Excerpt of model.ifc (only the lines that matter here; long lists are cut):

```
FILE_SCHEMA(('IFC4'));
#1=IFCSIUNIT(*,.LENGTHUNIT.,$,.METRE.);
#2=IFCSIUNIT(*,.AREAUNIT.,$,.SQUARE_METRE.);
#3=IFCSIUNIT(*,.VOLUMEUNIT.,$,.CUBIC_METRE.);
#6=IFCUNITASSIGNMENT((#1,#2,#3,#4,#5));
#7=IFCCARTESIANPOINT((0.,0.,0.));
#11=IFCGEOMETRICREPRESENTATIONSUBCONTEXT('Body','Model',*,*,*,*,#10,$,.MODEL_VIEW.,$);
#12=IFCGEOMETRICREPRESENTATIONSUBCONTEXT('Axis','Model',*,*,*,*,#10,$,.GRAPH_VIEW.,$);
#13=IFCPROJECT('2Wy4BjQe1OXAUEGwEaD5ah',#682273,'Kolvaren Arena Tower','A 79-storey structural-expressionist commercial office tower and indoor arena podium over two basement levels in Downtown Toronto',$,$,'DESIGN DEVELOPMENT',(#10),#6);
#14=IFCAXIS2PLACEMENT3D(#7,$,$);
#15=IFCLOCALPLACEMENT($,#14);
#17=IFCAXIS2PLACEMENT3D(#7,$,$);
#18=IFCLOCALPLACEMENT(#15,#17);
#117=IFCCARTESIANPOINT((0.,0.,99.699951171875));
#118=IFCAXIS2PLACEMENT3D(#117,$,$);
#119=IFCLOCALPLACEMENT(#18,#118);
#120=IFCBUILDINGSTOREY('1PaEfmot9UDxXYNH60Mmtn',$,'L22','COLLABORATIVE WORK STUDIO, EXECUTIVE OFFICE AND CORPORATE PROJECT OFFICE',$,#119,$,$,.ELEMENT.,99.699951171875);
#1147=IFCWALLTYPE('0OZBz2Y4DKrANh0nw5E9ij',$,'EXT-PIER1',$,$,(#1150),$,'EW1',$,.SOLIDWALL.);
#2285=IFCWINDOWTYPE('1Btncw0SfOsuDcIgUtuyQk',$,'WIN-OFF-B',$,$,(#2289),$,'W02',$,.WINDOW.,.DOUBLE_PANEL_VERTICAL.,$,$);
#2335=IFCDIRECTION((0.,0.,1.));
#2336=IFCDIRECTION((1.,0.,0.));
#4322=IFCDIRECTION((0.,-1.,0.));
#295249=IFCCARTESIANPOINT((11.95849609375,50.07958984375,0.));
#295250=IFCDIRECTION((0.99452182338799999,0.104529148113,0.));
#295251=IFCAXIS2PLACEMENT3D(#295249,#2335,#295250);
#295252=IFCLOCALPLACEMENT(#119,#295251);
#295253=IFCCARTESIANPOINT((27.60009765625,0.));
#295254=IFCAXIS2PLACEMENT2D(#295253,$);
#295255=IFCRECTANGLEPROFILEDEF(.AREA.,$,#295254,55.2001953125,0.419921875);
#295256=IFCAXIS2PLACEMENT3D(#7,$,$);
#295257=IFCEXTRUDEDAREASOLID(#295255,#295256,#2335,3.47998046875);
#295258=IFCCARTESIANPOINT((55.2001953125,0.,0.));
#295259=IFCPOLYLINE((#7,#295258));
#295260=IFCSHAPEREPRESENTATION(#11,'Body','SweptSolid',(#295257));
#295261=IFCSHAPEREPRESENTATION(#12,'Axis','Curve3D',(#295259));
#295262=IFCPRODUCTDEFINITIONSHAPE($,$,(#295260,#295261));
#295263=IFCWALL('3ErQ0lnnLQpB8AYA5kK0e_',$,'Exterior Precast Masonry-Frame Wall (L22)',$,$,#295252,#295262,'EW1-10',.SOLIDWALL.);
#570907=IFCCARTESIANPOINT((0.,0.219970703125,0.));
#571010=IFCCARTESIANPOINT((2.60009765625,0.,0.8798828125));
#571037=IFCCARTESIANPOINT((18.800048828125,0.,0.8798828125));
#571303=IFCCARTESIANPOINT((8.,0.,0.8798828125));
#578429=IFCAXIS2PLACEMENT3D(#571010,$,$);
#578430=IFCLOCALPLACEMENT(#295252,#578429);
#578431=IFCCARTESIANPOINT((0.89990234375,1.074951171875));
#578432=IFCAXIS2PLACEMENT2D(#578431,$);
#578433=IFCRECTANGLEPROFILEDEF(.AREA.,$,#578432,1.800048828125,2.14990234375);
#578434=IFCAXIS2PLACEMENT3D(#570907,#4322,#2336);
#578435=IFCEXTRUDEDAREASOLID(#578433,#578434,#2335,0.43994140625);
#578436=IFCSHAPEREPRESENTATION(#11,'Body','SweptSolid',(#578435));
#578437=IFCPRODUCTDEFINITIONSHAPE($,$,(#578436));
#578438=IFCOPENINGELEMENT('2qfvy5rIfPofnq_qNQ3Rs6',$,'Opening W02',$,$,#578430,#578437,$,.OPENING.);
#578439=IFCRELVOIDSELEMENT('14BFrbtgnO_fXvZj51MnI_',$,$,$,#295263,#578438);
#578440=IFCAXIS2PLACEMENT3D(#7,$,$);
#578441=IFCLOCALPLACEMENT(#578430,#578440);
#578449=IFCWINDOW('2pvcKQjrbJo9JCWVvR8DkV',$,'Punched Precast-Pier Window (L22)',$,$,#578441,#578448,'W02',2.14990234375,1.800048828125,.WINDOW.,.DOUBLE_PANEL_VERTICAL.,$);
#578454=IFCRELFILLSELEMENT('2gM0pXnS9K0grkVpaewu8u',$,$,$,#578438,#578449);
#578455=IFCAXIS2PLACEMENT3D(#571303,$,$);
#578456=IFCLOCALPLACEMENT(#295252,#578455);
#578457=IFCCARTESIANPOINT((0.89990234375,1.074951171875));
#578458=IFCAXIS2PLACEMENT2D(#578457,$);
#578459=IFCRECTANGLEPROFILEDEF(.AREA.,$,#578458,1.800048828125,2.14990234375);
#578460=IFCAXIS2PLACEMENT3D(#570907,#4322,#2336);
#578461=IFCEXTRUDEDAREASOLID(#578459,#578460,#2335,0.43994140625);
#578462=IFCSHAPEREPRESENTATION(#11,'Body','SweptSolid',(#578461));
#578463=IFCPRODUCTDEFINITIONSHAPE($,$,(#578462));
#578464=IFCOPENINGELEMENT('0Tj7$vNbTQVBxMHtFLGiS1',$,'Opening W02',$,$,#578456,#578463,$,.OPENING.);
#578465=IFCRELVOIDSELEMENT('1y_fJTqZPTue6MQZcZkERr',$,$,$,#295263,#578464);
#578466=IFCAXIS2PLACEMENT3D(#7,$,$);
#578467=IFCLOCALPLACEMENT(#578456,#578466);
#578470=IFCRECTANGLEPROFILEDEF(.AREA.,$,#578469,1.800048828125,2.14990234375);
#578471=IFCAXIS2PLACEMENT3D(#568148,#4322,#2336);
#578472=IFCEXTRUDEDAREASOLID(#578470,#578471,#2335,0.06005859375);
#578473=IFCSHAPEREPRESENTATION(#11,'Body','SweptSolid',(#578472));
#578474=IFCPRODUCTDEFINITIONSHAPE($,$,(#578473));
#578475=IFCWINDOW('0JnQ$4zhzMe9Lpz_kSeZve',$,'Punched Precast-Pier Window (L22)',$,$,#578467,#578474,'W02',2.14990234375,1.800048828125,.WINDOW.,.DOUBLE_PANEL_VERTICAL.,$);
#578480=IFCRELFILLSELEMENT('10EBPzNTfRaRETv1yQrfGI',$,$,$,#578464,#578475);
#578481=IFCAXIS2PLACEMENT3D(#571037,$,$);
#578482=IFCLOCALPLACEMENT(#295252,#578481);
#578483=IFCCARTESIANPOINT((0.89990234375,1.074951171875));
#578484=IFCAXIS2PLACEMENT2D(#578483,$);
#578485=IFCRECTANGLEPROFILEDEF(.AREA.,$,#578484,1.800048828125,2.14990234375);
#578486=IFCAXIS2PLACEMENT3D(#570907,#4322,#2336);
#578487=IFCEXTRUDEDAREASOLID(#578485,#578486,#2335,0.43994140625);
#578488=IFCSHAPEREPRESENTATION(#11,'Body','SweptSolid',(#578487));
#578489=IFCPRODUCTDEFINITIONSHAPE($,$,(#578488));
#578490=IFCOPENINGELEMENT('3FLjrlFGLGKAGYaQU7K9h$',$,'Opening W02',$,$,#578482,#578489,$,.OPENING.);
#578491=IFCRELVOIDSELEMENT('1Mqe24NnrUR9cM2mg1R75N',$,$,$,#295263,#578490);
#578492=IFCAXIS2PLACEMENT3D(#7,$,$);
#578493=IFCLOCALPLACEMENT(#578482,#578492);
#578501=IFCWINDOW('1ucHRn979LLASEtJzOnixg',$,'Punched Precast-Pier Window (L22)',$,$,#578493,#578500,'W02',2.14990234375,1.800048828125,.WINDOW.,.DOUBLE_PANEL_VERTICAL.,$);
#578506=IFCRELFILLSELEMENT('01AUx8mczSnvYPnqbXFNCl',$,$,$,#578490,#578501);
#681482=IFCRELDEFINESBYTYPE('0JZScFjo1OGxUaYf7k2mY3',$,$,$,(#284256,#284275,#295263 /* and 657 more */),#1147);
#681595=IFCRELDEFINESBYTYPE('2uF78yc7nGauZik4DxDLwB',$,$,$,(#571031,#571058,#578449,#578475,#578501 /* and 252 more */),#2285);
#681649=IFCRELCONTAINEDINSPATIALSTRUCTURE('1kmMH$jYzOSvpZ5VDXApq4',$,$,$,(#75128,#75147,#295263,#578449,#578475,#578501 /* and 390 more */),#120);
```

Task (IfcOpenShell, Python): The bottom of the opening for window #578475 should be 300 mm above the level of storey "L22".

```python
import numpy as np
import ifcopenshell
import ifcopenshell.api.geometry
import ifcopenshell.geom
import ifcopenshell.util.element
import ifcopenshell.util.placement
import ifcopenshell.util.shape
import ifcopenshell.util.unit

model = ifcopenshell.open("model.ifc")
unit_scale = ifcopenshell.util.unit.calculate_unit_scale(model)

window = model.by_guid("0JnQ$4zhzMe9Lpz_kSeZve")
opening = window.FillsVoids[0].RelatingOpeningElement
storey = ifcopenshell.util.element.get_container(window, ifc_class="IfcBuildingStorey")
level = ifcopenshell.util.placement.get_local_placement(storey.ObjectPlacement)[2, 3]

# The opening's origin need not be at the sill, so measure its lowest point.
shape = ifcopenshell.geom.create_shape(ifcopenshell.geom.settings(), opening)
bottom = ifcopenshell.util.shape.get_shape_bottom_elevation(shape, shape.geometry) / unit_scale
dz = level + 0.3 / unit_scale - bottom

shift = np.array([0.0, 0.0, dz])
# The window is placed relative to its opening, so it follows when the opening moves.
matrix = ifcopenshell.util.placement.get_local_placement(opening.ObjectPlacement)
matrix[:3, 3] += shift
ifcopenshell.api.geometry.edit_object_placement(
    model, product=opening, matrix=matrix, is_si=False, should_transform_children=True
)

print(f"moved by {dz * unit_scale:+.3f} m")

model.write("model_updated.ifc")
```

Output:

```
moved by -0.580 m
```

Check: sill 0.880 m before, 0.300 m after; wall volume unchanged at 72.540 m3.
